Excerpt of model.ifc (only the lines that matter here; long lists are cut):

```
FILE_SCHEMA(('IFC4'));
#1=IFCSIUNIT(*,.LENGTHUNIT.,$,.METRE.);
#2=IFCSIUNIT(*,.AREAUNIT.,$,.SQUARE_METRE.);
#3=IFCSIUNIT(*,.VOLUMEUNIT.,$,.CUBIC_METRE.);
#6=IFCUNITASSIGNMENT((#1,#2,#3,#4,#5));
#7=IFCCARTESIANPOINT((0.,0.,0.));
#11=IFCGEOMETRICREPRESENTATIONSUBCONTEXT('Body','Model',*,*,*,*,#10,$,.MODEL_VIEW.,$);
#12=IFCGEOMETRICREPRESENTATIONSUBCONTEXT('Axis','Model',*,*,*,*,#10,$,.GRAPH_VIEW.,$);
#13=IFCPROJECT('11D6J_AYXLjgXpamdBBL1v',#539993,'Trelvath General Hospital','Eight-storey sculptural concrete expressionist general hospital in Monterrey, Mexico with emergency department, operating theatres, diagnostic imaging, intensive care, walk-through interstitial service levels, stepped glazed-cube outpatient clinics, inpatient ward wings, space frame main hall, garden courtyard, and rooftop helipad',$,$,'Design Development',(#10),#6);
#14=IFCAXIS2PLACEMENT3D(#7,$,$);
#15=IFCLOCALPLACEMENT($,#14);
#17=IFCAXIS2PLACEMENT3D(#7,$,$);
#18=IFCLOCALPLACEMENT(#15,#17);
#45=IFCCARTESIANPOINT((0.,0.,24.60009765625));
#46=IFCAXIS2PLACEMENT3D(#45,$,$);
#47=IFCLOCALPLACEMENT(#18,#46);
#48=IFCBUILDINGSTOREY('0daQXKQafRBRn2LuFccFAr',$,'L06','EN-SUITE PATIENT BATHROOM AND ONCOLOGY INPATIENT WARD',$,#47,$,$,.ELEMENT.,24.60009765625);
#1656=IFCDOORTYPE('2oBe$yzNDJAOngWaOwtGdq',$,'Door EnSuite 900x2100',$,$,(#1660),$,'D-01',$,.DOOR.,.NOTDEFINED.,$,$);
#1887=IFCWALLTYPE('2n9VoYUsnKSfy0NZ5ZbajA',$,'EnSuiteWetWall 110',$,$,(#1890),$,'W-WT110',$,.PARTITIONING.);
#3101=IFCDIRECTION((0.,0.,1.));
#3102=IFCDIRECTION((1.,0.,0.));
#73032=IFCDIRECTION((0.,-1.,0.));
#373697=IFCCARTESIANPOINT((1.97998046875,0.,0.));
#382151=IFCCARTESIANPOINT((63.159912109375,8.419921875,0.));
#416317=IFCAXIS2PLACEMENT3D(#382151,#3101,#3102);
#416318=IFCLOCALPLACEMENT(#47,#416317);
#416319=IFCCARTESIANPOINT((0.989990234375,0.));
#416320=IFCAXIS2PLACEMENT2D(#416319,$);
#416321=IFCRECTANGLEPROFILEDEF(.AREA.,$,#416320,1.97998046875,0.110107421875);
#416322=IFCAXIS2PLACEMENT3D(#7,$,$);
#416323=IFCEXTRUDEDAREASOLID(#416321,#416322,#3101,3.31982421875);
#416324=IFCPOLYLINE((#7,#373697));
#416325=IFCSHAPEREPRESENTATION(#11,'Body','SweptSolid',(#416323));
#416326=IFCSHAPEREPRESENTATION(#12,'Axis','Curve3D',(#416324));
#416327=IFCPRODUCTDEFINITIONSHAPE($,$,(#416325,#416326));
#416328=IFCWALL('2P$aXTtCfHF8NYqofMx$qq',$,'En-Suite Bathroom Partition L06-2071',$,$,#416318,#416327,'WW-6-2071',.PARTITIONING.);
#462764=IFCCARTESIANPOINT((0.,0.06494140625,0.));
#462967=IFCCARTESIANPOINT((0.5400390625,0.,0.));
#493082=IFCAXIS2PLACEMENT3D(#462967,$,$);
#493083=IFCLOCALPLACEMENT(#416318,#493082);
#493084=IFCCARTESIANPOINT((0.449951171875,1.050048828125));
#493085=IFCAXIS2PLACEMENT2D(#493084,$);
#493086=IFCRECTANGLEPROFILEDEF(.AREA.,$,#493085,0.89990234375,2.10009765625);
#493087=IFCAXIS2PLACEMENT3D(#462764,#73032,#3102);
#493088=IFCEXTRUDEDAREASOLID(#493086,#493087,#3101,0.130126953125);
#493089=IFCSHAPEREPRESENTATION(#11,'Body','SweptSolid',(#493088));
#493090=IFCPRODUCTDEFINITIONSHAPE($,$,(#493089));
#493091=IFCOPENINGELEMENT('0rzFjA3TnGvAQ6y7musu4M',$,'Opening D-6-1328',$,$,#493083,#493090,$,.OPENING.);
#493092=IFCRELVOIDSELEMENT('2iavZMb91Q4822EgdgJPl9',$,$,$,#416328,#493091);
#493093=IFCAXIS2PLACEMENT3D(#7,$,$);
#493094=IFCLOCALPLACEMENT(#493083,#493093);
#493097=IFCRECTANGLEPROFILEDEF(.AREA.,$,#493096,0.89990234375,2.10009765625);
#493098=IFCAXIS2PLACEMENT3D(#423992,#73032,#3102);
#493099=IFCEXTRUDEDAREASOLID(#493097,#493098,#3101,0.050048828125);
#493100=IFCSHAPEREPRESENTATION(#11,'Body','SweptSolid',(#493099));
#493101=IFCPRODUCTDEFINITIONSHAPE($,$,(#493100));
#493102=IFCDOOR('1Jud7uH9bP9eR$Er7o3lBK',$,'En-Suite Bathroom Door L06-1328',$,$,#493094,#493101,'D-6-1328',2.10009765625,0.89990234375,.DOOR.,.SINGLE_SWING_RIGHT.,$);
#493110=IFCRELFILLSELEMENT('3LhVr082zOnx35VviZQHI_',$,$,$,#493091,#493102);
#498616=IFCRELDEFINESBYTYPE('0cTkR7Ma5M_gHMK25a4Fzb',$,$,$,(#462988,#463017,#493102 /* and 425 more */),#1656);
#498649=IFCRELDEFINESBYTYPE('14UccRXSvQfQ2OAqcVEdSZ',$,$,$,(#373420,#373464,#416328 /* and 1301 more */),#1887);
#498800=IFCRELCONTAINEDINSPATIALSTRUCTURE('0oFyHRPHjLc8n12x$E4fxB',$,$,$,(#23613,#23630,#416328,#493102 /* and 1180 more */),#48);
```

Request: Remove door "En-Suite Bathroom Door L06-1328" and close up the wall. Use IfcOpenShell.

```python
import ifcopenshell
import ifcopenshell.api.feature
import ifcopenshell.api.root
import ifcopenshell.geom
import ifcopenshell.util.shape

model = ifcopenshell.open("model.ifc")
settings = ifcopenshell.geom.settings()


def volume(element):
    """Net volume in cubic metres, openings subtracted."""
    shape = ifcopenshell.geom.create_shape(settings, element)
    return ifcopenshell.util.shape.get_volume(shape.geometry)


door = model.by_guid("1Jud7uH9bP9eR$Er7o3lBK")
opening = door.FillsVoids[0].RelatingOpeningElement
wall = opening.VoidsElements[0].RelatingBuildingElement
before = volume(wall)

ifcopenshell.api.root.remove_product(model, product=door)
ifcopenshell.api.feature.remove_feature(model, feature=opening)

after = volume(wall)

print(f"wall volume {before:.3f} -> {after:.3f} m3")

model.write("model_edited.ifc")
```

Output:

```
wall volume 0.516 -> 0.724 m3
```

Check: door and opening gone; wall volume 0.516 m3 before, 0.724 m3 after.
